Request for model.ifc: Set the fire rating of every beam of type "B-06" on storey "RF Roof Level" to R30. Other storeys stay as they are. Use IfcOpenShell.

First a look at what the model holds.

```python
import ifcopenshell
import ifcopenshell.util.element

model = ifcopenshell.open("model.ifc")
print(model.schema)
storey = next(s for s in model.by_type("IfcBuildingStorey") if s.Name == "RF Roof Level")
beams = [e for e in ifcopenshell.util.element.get_decomposition(storey) if e.is_a("IfcBeam")]
seen = {}
for e in beams:
    element_type = ifcopenshell.util.element.get_type(e)
    key = (element_type.Name if element_type != e and element_type else None, ifcopenshell.util.element.get_pset(e, "Pset_BeamCommon", "FireRating"))
    seen[key] = seen.get(key, 0) + 1
for (name, value), count in sorted(seen.items(), key=str):
    print(count, "x", name, "|", value)
```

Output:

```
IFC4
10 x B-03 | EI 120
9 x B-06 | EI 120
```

```python
import ifcopenshell
import ifcopenshell.api.pset
import ifcopenshell.util.element

model = ifcopenshell.open("model.ifc")

storey = next(s for s in model.by_type("IfcBuildingStorey") if s.Name == "RF Roof Level")
beams = [e for e in ifcopenshell.util.element.get_decomposition(storey) if e.is_a("IfcBeam")]

count = 0
for e in beams:
    element_type = ifcopenshell.util.element.get_type(e)
    if element_type in (None, e) or element_type.Name != "B-06":
        continue
    # add_pset returns the element's existing set when there is one.
    pset = ifcopenshell.api.pset.add_pset(model, product=e, name="Pset_BeamCommon")
    ifcopenshell.api.pset.edit_pset(model, pset=pset, properties={"FireRating": "R30"})
    count += 1

print(count, "beams updated")

model.write("model_rev.ifc")
```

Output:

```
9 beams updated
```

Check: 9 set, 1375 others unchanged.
